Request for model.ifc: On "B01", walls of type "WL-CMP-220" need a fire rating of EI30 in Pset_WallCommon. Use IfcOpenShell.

First a look at what the model holds.

```python
import ifcopenshell
import ifcopenshell.util.element

model = ifcopenshell.open("model.ifc")
print(model.schema)
storey = next(s for s in model.by_type("IfcBuildingStorey") if s.Name == "B01")
walls = [e for e in ifcopenshell.util.element.get_decomposition(storey) if e.is_a("IfcWall")]
seen = {}
for e in walls:
    element_type = ifcopenshell.util.element.get_type(e)
    key = (element_type.Name if element_type != e and element_type else None, ifcopenshell.util.element.get_pset(e, "Pset_WallCommon", "FireRating"))
    seen[key] = seen.get(key, 0) + 1
for (name, value), count in sorted(seen.items(), key=str):
    print(count, "x", name, "|", value)
```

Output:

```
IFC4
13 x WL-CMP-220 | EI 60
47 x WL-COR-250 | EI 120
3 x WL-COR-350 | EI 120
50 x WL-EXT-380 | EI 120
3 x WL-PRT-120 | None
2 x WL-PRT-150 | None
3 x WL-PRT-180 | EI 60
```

```python
import ifcopenshell
import ifcopenshell.api.pset
import ifcopenshell.util.element

model = ifcopenshell.open("model.ifc")

storey = next(s for s in model.by_type("IfcBuildingStorey") if s.Name == "B01")
walls = [e for e in ifcopenshell.util.element.get_decomposition(storey) if e.is_a("IfcWall")]

count = 0
for e in walls:
    element_type = ifcopenshell.util.element.get_type(e)
    if element_type in (None, e) or element_type.Name != "WL-CMP-220":
        continue
    # add_pset returns the element's existing set when there is one.
    pset = ifcopenshell.api.pset.add_pset(model, product=e, name="Pset_WallCommon")
    ifcopenshell.api.pset.edit_pset(model, pset=pset, properties={"FireRating": "EI30"})
    count += 1

print(count, "walls updated")

model.write("model_v2.ifc")
```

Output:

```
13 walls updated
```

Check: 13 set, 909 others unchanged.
